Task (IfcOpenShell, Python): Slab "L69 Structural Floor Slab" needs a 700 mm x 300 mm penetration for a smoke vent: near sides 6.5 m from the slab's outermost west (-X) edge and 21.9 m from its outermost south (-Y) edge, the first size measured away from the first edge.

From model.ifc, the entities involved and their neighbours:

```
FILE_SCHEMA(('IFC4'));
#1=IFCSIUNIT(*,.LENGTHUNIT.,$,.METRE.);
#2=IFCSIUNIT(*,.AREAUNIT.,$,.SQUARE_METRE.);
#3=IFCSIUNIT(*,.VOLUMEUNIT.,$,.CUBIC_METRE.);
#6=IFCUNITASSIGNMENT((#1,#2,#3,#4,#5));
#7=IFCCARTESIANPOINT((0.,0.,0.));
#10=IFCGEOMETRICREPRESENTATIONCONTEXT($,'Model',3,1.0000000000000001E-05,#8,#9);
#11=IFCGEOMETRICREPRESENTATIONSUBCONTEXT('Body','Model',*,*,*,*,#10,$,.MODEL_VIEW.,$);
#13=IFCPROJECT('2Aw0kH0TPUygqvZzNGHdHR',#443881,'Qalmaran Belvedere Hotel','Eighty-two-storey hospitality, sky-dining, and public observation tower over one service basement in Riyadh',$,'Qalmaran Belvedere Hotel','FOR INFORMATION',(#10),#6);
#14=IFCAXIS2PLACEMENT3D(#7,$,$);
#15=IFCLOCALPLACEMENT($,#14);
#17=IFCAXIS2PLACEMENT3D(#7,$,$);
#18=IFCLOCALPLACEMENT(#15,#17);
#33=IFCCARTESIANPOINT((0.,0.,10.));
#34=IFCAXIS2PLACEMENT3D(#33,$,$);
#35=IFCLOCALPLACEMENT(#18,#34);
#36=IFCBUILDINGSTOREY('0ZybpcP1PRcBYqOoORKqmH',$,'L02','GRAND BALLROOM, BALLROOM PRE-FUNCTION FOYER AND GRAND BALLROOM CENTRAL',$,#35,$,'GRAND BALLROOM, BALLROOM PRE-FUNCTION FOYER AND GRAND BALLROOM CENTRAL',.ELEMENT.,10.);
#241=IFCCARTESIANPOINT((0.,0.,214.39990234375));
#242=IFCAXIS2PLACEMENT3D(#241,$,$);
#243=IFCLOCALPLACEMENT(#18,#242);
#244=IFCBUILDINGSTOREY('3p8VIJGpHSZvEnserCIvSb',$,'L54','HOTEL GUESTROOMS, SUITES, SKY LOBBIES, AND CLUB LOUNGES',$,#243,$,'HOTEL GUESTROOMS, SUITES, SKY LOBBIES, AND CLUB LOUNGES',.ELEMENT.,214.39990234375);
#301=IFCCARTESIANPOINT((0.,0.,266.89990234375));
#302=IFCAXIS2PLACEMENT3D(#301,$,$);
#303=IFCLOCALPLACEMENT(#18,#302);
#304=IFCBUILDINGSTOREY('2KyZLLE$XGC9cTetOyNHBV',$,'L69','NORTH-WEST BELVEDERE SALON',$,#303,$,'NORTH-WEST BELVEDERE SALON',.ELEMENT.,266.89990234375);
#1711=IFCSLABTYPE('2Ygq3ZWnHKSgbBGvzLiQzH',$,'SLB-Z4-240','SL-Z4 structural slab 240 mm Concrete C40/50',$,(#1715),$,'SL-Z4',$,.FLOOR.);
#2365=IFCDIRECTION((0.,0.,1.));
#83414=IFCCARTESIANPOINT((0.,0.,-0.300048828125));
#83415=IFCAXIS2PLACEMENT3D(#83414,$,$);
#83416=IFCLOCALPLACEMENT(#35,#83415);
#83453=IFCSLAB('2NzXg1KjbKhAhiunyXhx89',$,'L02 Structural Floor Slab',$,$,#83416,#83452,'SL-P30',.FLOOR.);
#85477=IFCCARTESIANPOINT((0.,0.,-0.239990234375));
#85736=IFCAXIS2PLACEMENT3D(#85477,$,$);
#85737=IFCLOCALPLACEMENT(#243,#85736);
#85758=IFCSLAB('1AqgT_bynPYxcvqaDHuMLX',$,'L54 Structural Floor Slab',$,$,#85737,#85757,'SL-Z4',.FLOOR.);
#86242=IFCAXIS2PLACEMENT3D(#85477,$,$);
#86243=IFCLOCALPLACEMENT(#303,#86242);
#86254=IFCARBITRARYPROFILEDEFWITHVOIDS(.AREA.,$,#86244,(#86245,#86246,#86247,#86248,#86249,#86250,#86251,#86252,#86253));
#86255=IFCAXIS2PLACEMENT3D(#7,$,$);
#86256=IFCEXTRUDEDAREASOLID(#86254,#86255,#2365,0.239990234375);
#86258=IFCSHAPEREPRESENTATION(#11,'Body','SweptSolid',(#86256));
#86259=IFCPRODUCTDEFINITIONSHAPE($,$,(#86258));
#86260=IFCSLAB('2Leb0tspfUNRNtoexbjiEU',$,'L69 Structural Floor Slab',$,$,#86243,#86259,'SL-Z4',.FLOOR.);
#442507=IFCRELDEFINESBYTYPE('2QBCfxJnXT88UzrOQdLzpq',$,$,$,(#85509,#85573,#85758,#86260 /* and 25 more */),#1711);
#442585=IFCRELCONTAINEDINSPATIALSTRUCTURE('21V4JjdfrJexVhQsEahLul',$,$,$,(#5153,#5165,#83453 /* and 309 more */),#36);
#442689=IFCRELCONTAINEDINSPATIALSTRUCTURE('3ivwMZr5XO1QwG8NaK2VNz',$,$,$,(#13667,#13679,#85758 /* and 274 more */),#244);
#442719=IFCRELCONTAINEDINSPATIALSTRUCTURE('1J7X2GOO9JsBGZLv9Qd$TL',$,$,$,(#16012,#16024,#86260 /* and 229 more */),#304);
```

```python
import numpy as np
import ifcopenshell
import ifcopenshell.api.feature
import ifcopenshell.api.geometry
import ifcopenshell.api.root
import ifcopenshell.geom
import ifcopenshell.util.placement
import ifcopenshell.util.representation
import ifcopenshell.util.shape
import ifcopenshell.util.unit

model = ifcopenshell.open("model.ifc")
unit_scale = ifcopenshell.util.unit.calculate_unit_scale(model)
settings = ifcopenshell.geom.settings()


def volume(element):
    """Net volume in cubic metres, openings subtracted."""
    shape = ifcopenshell.geom.create_shape(settings, element)
    return ifcopenshell.util.shape.get_volume(shape.geometry)


slab = model.by_guid("2Leb0tspfUNRNtoexbjiEU")
before = volume(slab)

# Extent in the slab's own axes, in metres. The edges named are its -X and -Y sides.
slab_shape = ifcopenshell.geom.create_shape(settings, slab)
vertices = ifcopenshell.util.shape.get_vertices(slab_shape.geometry)
x_min, y_min, bottom = vertices.min(axis=0)
top = vertices[:, 2].max()

opening = ifcopenshell.api.root.create_entity(model, ifc_class="IfcOpeningElement", name="Smoke vent opening", predefined_type="OPENING")
context = ifcopenshell.util.representation.get_context(model, "Model", "Body", "MODEL_VIEW")
width, depth = 0.7, 0.3
outline = [(0.0, 0.0), (width, 0.0), (width, depth), (0.0, depth), (0.0, 0.0)]
# Overshoot both faces by 50 mm so the cut is clean.
shape = ifcopenshell.api.geometry.add_slab_representation(
    model, context=context, depth=top - bottom + 0.1, polyline=outline
)
ifcopenshell.api.geometry.assign_representation(model, product=opening, representation=shape)

matrix = ifcopenshell.util.placement.get_local_placement(slab.ObjectPlacement)
matrix[:, 3] = matrix @ np.append(np.array([x_min + 6.5, y_min + 21.9, bottom - 0.05]) / unit_scale, 1.0)
ifcopenshell.api.geometry.edit_object_placement(model, product=opening, matrix=matrix, is_si=False)
ifcopenshell.api.feature.add_feature(model, feature=opening, element=slab)

after = volume(slab)

print(f"slab volume {before:.3f} -> {after:.3f} m3")

model.write("model_v2.ifc")
```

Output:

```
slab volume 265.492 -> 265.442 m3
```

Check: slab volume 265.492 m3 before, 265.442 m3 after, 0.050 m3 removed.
